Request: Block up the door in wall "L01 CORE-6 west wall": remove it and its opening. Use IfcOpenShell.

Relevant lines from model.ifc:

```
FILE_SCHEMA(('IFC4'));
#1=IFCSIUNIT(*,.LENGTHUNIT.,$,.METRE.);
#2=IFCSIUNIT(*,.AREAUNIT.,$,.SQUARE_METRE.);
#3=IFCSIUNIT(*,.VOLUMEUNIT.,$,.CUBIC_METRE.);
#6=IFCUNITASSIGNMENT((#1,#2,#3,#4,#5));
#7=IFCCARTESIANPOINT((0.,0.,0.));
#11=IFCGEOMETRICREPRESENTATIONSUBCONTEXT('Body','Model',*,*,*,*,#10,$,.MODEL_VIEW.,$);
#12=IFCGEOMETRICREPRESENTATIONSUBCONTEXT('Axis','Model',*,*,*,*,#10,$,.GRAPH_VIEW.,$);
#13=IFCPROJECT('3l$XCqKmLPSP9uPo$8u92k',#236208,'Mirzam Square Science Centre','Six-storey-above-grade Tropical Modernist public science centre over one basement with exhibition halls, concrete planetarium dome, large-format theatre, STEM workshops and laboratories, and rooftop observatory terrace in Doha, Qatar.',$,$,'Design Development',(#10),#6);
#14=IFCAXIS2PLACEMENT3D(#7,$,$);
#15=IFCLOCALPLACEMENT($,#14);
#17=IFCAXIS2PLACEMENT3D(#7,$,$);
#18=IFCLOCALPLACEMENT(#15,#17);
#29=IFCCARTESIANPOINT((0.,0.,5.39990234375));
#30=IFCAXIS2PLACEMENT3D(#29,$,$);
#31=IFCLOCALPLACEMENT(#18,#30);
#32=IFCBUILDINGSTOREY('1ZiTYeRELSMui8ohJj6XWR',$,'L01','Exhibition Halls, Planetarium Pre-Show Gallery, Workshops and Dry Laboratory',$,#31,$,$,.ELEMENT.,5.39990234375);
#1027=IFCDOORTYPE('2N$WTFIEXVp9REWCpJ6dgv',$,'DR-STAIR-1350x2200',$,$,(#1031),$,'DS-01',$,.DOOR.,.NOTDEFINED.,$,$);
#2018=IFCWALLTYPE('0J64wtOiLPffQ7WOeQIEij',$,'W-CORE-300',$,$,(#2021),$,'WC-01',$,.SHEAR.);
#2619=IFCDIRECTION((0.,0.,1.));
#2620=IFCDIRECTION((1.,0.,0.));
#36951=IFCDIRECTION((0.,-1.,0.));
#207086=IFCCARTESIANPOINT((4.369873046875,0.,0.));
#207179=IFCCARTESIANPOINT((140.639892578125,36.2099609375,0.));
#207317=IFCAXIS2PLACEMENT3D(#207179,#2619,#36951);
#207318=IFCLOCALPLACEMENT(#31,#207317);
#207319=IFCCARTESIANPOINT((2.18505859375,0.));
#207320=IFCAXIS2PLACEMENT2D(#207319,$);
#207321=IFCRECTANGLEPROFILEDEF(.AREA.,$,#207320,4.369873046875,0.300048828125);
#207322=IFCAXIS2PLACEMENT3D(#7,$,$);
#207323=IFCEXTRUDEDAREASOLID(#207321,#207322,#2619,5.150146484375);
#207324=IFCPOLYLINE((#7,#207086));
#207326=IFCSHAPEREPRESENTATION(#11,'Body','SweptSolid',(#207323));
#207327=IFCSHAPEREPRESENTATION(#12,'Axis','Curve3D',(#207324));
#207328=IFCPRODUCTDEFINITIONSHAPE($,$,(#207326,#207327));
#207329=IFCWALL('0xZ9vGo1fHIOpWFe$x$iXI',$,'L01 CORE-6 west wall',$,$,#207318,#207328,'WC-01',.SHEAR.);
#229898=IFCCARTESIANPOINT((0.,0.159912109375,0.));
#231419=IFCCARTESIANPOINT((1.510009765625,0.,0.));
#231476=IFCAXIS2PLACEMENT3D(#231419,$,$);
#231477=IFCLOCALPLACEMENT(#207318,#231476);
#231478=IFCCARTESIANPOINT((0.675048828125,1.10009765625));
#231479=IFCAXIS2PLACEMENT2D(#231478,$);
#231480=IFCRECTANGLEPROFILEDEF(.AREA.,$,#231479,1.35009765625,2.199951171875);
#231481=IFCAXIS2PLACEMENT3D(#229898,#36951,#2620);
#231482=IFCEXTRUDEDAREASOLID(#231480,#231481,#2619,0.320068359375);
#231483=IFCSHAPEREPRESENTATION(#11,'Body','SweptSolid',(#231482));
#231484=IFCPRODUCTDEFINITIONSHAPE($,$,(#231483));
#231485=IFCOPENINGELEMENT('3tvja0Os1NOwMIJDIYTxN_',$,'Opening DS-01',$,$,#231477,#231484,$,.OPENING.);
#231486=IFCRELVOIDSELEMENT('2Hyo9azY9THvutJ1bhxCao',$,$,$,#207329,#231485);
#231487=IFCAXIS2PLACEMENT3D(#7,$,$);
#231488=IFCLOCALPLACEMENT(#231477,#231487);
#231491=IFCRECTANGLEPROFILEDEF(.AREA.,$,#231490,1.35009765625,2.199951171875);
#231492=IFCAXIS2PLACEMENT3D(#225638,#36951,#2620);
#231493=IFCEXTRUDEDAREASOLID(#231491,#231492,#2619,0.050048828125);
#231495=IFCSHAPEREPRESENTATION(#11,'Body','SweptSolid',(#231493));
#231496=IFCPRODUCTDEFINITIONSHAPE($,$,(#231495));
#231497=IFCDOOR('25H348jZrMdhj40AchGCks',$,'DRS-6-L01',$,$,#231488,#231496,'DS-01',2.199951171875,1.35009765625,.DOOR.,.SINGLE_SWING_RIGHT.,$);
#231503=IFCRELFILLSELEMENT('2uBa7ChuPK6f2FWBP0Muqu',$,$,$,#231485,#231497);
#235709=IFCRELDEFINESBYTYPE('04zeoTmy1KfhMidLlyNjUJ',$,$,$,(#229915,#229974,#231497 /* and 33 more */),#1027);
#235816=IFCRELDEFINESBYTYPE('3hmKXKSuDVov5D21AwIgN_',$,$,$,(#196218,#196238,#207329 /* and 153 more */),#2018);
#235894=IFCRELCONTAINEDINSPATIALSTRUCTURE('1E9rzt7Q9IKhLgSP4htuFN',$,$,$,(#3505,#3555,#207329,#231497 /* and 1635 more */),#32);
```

```python
import ifcopenshell
import ifcopenshell.api.feature
import ifcopenshell.api.root
import ifcopenshell.geom
import ifcopenshell.util.shape

model = ifcopenshell.open("model.ifc")
settings = ifcopenshell.geom.settings()


def volume(element):
    """Net volume in cubic metres, openings subtracted."""
    shape = ifcopenshell.geom.create_shape(settings, element)
    return ifcopenshell.util.shape.get_volume(shape.geometry)


door = model.by_guid("25H348jZrMdhj40AchGCks")
opening = door.FillsVoids[0].RelatingOpeningElement
wall = opening.VoidsElements[0].RelatingBuildingElement
before = volume(wall)

ifcopenshell.api.root.remove_product(model, product=door)
ifcopenshell.api.feature.remove_feature(model, feature=opening)

after = volume(wall)

print(f"wall volume {before:.3f} -> {after:.3f} m3")

model.write("model-out.ifc")
```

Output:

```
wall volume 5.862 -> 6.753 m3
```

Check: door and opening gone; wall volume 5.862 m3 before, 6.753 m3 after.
